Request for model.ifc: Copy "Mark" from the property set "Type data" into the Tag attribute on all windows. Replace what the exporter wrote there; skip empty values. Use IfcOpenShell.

First a look at what the model holds.

```python
import ifcopenshell
import ifcopenshell.util.element

model = ifcopenshell.open("model.ifc")
print(model.schema)
windows = model.by_type("IfcWindow")
print(len(windows), "windows")
for e in windows[:8]:
    source = ifcopenshell.util.element.get_pset(e, "Type data", "Mark")
    target = e.Tag
    print(e.id(), repr(source), repr(target), sep=" | ")
```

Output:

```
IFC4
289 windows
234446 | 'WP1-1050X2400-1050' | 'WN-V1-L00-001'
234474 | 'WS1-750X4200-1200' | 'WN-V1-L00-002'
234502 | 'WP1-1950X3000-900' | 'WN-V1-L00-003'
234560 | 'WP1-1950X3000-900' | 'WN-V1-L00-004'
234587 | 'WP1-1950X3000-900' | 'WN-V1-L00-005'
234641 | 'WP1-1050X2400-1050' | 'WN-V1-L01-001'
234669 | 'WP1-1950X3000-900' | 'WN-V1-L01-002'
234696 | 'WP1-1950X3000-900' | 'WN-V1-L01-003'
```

```python
import ifcopenshell
import ifcopenshell.util.element

model = ifcopenshell.open("model.ifc")

count = 0
for e in model.by_type("IfcWindow"):
    value = ifcopenshell.util.element.get_pset(e, "Type data", "Mark")
    current = e.Tag
    if not value or not value.strip() or current == value:
        continue
    e.Tag = value
    count += 1

print(count, "windows updated")

model.write("model_rev.ifc")
```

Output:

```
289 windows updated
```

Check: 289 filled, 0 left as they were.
